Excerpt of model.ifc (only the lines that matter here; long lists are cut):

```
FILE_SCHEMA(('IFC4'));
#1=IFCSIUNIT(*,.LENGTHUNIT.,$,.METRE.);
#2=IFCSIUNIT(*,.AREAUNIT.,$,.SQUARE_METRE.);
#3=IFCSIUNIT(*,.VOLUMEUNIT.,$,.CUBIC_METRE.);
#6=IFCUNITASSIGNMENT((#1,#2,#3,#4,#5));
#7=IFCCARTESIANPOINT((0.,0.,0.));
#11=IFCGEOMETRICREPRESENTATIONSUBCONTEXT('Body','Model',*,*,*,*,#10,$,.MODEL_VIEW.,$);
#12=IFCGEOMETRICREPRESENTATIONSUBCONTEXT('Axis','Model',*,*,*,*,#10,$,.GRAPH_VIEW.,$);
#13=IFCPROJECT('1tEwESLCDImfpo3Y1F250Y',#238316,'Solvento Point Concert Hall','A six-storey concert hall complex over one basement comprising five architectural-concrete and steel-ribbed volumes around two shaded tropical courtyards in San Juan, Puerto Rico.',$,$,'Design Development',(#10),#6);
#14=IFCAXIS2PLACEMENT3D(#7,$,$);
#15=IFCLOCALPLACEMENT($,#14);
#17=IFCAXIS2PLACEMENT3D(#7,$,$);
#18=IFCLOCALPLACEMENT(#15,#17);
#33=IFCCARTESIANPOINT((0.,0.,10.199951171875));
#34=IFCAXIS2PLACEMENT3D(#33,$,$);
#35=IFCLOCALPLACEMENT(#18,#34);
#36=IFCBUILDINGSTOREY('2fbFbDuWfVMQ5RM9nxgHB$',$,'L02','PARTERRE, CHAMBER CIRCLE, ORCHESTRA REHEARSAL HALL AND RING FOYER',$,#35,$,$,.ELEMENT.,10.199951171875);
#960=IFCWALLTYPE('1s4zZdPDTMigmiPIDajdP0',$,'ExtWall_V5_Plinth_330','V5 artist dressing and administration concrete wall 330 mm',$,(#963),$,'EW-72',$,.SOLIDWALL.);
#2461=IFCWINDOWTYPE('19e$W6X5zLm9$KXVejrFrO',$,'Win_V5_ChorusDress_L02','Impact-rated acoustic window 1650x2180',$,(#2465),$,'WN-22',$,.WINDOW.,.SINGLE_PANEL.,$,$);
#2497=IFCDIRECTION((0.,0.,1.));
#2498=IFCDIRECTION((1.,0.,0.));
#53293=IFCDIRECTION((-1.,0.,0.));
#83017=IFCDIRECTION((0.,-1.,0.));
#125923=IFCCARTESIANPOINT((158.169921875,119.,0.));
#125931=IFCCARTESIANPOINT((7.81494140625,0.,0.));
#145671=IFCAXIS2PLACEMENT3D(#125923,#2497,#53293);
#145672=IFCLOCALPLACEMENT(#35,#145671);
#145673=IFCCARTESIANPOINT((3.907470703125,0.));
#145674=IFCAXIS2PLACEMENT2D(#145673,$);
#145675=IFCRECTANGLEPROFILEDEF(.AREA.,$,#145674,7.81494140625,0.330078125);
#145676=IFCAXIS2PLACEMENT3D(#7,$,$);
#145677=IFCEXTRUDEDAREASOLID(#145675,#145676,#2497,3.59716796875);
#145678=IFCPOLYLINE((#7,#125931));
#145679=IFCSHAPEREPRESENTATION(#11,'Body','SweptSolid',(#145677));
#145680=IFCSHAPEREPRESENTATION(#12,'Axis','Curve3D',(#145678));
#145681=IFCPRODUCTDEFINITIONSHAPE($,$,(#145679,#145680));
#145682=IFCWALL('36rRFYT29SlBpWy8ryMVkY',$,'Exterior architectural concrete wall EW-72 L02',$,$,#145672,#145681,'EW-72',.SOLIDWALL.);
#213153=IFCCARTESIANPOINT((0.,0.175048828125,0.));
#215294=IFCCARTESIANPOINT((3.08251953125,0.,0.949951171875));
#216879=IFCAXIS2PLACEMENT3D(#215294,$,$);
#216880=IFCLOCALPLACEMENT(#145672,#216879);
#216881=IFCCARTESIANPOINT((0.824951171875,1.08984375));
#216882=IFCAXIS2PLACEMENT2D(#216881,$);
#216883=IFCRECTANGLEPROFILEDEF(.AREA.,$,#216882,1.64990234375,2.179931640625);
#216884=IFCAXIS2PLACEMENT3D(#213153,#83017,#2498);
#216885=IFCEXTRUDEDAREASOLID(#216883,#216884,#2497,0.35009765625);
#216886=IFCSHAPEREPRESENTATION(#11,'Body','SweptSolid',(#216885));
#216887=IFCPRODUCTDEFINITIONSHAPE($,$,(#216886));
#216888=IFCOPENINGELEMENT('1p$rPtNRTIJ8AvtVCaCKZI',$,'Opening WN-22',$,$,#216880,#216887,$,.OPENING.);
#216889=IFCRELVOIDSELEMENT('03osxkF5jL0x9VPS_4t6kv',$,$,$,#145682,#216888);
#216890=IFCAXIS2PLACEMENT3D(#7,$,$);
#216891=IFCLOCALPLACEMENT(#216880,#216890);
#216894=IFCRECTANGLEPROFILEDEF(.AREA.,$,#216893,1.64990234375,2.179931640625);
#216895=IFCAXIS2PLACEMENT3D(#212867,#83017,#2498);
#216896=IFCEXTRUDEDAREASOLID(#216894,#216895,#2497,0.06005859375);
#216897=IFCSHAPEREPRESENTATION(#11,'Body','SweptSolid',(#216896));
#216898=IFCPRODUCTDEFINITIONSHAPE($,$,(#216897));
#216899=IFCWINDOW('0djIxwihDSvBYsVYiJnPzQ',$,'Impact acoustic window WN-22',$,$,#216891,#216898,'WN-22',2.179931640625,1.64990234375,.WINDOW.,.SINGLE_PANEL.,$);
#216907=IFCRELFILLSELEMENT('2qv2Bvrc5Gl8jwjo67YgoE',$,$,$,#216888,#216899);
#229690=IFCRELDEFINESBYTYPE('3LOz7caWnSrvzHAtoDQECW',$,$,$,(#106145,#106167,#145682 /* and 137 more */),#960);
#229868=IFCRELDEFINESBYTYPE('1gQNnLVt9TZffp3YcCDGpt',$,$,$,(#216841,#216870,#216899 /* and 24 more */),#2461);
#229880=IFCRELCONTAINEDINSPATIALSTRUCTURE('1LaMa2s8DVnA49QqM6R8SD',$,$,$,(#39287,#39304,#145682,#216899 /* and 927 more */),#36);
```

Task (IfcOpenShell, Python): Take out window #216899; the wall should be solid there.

```python
import ifcopenshell
import ifcopenshell.api.feature
import ifcopenshell.api.root
import ifcopenshell.geom
import ifcopenshell.util.shape

model = ifcopenshell.open("model.ifc")
settings = ifcopenshell.geom.settings()


def volume(element):
    """Net volume in cubic metres, openings subtracted."""
    shape = ifcopenshell.geom.create_shape(settings, element)
    return ifcopenshell.util.shape.get_volume(shape.geometry)


window = model.by_guid("0djIxwihDSvBYsVYiJnPzQ")
opening = window.FillsVoids[0].RelatingOpeningElement
wall = opening.VoidsElements[0].RelatingBuildingElement
before = volume(wall)

ifcopenshell.api.root.remove_product(model, product=window)
ifcopenshell.api.feature.remove_feature(model, feature=opening)

after = volume(wall)

print(f"wall volume {before:.3f} -> {after:.3f} m3")

model.write("model_v2.ifc")
```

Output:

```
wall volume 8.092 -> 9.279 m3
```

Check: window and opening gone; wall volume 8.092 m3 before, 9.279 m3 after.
